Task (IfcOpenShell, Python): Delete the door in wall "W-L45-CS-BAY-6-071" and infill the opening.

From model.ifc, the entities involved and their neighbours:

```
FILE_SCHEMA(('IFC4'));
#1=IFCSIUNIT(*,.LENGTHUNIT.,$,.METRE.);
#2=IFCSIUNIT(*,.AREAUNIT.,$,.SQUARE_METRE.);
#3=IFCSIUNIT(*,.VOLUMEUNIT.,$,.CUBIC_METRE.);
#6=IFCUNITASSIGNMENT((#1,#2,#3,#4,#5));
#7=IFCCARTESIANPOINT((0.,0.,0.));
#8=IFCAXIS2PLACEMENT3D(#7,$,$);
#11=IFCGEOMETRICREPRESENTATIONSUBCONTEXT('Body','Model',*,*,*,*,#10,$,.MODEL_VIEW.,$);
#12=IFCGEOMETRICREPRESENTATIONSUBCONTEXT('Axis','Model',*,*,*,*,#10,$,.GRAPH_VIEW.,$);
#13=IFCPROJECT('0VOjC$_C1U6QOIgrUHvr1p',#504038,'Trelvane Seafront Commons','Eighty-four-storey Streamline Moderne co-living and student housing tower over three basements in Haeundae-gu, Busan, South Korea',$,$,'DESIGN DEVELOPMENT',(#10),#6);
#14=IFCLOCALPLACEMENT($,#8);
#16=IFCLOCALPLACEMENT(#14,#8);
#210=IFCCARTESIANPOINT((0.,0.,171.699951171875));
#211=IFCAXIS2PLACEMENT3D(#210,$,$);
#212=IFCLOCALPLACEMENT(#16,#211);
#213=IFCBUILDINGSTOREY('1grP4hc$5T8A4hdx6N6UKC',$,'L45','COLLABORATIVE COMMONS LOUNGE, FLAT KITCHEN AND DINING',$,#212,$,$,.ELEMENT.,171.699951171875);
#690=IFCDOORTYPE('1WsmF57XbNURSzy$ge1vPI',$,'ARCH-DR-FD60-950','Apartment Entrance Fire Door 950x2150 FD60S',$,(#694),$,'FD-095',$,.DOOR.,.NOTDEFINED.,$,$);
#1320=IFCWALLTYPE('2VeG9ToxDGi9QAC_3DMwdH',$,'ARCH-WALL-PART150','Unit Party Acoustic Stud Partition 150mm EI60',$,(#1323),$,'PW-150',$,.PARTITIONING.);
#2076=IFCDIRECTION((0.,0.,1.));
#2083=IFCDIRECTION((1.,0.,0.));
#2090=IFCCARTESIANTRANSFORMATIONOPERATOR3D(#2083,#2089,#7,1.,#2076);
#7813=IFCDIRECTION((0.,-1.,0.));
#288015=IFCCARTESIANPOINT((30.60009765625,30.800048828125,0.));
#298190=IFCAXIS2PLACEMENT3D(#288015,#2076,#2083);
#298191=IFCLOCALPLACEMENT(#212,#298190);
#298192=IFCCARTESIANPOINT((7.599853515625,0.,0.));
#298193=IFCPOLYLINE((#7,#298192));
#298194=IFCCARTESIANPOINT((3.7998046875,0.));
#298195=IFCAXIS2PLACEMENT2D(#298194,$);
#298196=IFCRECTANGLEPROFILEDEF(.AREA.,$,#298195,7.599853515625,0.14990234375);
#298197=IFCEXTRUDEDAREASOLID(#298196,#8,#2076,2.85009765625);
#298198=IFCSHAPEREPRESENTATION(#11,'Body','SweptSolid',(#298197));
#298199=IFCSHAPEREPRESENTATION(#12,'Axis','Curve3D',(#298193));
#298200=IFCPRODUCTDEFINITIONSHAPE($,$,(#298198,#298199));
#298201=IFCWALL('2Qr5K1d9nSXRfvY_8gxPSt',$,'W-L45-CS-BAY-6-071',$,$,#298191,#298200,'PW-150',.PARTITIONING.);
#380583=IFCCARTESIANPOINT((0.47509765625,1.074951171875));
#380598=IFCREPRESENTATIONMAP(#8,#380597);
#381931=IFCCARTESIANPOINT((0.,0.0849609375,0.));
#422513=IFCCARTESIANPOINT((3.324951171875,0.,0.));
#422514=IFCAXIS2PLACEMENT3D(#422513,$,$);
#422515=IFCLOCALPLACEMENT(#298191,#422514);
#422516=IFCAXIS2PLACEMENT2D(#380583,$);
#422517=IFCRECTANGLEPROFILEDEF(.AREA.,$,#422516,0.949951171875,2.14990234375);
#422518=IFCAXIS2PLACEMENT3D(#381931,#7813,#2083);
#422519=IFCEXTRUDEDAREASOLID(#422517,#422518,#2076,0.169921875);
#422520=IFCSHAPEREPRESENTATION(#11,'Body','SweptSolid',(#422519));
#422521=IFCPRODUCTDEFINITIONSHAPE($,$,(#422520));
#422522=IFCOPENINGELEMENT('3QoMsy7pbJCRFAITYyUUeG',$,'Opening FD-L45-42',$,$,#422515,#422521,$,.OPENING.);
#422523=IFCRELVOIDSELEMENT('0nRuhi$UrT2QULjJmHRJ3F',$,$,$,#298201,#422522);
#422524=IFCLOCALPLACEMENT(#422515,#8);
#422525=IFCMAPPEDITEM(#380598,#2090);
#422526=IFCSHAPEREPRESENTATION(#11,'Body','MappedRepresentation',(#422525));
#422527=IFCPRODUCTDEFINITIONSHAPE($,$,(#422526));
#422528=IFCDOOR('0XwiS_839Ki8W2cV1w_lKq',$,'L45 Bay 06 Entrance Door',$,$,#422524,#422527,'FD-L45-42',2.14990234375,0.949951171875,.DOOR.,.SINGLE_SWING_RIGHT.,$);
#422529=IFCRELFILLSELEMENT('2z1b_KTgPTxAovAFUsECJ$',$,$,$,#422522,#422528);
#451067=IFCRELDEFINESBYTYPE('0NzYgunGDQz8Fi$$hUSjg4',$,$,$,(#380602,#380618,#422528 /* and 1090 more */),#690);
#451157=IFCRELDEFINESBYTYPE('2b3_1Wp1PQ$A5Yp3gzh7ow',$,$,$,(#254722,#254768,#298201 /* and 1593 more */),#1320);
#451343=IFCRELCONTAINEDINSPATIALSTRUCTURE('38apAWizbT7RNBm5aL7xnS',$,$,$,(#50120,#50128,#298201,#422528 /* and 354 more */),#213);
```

```python
import ifcopenshell
import ifcopenshell.api.feature
import ifcopenshell.api.root
import ifcopenshell.geom
import ifcopenshell.util.shape

model = ifcopenshell.open("model.ifc")
settings = ifcopenshell.geom.settings()


def volume(element):
    """Net volume in cubic metres, openings subtracted."""
    shape = ifcopenshell.geom.create_shape(settings, element)
    return ifcopenshell.util.shape.get_volume(shape.geometry)


door = model.by_guid("0XwiS_839Ki8W2cV1w_lKq")
opening = door.FillsVoids[0].RelatingOpeningElement
wall = opening.VoidsElements[0].RelatingBuildingElement
before = volume(wall)

ifcopenshell.api.root.remove_product(model, product=door)
ifcopenshell.api.feature.remove_feature(model, feature=opening)

after = volume(wall)

print(f"wall volume {before:.3f} -> {after:.3f} m3")

model.write("model_updated.ifc")
```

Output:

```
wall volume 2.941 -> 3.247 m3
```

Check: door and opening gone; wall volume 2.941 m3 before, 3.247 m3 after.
